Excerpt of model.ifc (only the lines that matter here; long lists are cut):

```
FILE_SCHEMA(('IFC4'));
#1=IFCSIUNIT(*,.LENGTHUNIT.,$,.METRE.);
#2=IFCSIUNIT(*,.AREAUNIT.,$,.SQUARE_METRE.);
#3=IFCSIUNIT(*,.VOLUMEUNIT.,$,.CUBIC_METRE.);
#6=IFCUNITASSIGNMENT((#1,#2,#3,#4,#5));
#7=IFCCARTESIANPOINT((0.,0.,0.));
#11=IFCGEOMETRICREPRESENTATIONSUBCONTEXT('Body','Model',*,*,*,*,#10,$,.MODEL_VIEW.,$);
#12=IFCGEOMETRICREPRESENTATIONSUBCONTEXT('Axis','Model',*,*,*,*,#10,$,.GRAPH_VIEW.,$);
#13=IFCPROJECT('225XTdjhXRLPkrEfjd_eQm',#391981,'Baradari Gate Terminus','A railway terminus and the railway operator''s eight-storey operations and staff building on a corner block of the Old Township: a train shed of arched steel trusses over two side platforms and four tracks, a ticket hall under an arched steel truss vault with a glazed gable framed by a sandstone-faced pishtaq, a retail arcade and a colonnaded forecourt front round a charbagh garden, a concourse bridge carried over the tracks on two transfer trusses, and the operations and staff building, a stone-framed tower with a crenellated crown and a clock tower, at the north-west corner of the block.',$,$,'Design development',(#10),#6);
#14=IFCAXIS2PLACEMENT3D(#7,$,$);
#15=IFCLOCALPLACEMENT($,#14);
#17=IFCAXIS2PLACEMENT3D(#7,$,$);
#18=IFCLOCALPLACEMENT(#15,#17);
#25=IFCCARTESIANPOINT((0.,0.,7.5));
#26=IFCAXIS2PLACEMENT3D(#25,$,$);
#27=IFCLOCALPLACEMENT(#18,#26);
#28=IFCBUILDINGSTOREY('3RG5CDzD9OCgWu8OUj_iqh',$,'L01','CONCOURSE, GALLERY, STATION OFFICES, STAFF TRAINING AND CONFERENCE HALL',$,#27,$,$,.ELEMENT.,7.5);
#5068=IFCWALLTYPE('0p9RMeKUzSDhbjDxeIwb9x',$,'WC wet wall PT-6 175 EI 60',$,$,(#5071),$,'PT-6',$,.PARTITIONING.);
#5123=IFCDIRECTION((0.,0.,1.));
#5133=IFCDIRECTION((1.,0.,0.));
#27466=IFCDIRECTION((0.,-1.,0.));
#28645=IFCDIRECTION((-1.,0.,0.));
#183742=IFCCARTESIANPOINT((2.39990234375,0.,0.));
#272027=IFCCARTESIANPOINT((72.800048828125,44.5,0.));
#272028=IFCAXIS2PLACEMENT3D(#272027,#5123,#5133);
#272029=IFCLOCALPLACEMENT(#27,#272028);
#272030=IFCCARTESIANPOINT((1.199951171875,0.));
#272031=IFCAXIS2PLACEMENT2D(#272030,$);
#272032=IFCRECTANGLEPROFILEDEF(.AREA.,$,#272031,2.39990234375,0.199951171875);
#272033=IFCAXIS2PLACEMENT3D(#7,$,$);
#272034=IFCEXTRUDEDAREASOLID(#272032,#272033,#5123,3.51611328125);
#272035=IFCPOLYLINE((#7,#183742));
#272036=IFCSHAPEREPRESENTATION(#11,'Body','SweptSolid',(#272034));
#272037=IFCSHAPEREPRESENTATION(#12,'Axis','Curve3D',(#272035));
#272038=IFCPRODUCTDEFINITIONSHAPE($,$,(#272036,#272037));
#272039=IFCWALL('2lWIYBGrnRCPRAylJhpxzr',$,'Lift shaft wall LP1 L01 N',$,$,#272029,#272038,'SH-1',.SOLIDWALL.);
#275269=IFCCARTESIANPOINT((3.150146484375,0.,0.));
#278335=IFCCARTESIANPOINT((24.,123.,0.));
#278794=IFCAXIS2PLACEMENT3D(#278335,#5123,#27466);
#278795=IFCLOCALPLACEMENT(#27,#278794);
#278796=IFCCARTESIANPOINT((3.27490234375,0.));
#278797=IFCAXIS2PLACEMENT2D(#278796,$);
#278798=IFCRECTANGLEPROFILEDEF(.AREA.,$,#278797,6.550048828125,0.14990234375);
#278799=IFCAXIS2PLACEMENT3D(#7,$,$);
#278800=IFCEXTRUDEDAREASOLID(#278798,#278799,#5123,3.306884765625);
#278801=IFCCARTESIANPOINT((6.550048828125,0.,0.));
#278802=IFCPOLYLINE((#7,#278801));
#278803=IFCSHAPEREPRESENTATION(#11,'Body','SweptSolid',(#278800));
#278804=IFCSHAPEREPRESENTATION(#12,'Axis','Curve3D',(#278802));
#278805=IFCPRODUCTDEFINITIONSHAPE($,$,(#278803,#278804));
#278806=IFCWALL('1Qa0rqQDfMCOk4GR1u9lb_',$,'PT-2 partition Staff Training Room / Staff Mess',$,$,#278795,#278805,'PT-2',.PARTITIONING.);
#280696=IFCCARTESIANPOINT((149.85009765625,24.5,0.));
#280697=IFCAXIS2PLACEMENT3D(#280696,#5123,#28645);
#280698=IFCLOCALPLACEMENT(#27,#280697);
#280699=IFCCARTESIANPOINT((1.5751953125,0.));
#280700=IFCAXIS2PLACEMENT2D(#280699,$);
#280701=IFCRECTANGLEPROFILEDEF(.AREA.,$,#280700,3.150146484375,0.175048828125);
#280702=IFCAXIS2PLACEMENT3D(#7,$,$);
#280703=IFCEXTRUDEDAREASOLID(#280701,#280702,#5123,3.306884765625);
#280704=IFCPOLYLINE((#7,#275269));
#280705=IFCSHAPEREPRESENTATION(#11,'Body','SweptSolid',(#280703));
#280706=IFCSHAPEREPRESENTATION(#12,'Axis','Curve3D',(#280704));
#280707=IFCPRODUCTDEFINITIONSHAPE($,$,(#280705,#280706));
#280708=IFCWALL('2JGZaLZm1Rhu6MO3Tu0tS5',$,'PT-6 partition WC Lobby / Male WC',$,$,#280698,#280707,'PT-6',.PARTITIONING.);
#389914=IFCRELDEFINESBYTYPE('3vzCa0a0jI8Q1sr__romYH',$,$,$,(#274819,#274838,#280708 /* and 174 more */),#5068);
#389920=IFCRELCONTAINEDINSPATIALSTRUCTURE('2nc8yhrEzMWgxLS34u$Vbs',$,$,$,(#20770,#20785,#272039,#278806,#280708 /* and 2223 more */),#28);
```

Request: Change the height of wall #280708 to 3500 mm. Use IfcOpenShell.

```python
import ifcopenshell
import ifcopenshell.geom
import ifcopenshell.util.representation
import ifcopenshell.util.shape
import ifcopenshell.util.unit

model = ifcopenshell.open("model.ifc")
unit_scale = ifcopenshell.util.unit.calculate_unit_scale(model)
settings = ifcopenshell.geom.settings()


def volume(element):
    """Net volume in cubic metres, openings subtracted."""
    shape = ifcopenshell.geom.create_shape(settings, element)
    return ifcopenshell.util.shape.get_volume(shape.geometry)


wall = model.by_guid("2JGZaLZm1Rhu6MO3Tu0tS5")
before = volume(wall)

body = ifcopenshell.util.representation.get_representation(wall, "Model", "Body")
solid = body.Items[0]
old_height = solid.Depth
solid.Depth = 3.5 / unit_scale
after = volume(wall)

print(f"height {old_height:g} -> {solid.Depth:g}, volume {before:.3f} -> {after:.3f} m3")

model.write("model_v2.ifc")
```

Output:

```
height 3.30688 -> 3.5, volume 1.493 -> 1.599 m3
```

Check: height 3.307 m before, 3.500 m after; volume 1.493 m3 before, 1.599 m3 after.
